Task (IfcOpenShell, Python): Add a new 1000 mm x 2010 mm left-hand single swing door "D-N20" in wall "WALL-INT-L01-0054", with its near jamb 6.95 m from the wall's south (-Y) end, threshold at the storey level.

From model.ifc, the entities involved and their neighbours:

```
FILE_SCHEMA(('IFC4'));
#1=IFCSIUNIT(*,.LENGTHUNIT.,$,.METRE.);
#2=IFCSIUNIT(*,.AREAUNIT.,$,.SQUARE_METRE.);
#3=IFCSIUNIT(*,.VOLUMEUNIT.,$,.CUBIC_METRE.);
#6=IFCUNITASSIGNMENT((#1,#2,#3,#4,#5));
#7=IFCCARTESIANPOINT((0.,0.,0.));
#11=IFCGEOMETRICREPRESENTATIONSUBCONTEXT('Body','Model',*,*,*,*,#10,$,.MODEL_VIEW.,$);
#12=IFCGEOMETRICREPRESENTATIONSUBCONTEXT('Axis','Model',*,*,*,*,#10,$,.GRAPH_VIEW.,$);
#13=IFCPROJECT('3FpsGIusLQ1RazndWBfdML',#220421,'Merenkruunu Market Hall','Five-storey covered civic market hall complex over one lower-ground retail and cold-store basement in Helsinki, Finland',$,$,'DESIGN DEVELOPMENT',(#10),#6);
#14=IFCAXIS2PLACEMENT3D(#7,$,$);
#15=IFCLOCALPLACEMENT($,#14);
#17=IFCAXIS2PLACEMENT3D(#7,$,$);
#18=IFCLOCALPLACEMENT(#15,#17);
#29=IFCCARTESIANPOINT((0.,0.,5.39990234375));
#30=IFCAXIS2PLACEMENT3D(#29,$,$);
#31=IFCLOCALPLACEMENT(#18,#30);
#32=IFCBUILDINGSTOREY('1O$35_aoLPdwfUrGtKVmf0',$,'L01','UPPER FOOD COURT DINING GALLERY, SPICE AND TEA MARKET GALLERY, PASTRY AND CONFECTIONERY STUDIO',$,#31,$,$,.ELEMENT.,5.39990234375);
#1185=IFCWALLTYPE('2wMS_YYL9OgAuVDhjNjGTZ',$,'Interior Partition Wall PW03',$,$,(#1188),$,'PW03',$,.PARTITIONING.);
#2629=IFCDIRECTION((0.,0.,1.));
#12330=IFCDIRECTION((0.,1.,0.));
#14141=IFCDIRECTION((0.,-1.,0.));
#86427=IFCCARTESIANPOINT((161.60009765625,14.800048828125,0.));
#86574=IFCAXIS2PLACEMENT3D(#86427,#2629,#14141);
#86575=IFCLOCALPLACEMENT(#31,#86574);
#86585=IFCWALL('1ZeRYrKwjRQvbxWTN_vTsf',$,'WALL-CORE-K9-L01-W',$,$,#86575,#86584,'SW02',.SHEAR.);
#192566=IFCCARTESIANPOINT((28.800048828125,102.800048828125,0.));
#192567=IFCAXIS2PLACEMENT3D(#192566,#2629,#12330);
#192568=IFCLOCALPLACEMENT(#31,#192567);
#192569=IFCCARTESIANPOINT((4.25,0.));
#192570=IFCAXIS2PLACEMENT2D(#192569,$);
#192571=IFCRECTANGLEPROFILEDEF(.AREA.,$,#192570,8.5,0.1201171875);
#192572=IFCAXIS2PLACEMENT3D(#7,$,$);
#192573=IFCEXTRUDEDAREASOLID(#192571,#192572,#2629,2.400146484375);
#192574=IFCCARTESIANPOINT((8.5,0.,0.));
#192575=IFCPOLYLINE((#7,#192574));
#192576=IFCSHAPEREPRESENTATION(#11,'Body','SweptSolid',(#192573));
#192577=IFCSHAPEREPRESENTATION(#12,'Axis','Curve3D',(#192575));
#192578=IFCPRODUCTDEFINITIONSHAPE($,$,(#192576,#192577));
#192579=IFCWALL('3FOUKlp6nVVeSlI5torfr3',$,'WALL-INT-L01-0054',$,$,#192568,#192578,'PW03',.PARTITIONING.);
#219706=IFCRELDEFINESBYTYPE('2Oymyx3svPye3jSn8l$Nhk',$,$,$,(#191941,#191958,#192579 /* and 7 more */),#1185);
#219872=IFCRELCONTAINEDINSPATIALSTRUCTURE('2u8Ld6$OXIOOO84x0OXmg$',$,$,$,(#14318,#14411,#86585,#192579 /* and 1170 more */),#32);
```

```python
import numpy as np
import ifcopenshell
import ifcopenshell.api.feature
import ifcopenshell.api.geometry
import ifcopenshell.api.root
import ifcopenshell.api.spatial
import ifcopenshell.geom
import ifcopenshell.util.element
import ifcopenshell.util.placement
import ifcopenshell.util.representation
import ifcopenshell.util.shape
import ifcopenshell.util.unit

model = ifcopenshell.open("model.ifc")
unit_scale = ifcopenshell.util.unit.calculate_unit_scale(model)
settings = ifcopenshell.geom.settings()


def volume(element):
    """Net volume in cubic metres, openings subtracted."""
    shape = ifcopenshell.geom.create_shape(settings, element)
    return ifcopenshell.util.shape.get_volume(shape.geometry)


wall = model.by_id(192579)
storey = ifcopenshell.util.element.get_container(wall, ifc_class="IfcBuildingStorey")
context = ifcopenshell.util.representation.get_context(model, "Model", "Body", "MODEL_VIEW")
before = volume(wall)

width, height, from_end, sill = 1, 2.01, 6.95, 0.0  # metres

# The wall runs along its own X axis, and the end named is its -X end.
wall_shape = ifcopenshell.geom.create_shape(settings, wall)
x, y, z = ifcopenshell.util.shape.get_vertices(wall_shape.geometry).T
start = x.min() + from_end
face, thickness = float(y.min()), float(y.max() - y.min())
wall_matrix = ifcopenshell.util.placement.get_local_placement(wall.ObjectPlacement)
level = ifcopenshell.util.placement.get_local_placement(storey.ObjectPlacement)[2, 3]


def in_wall(x, y):
    """Placement at x, y metres in the wall's axes, at sill height."""
    matrix = wall_matrix.copy()
    matrix[:, 3] = wall_matrix @ np.array([x / unit_scale, y / unit_scale, 0.0, 1.0])
    matrix[2, 3] = level + sill / unit_scale
    return matrix


# Opening: a box that overshoots both wall faces by 50 mm.
opening = ifcopenshell.api.root.create_entity(model, ifc_class="IfcOpeningElement", predefined_type="OPENING")
box = ifcopenshell.api.geometry.add_wall_representation(
    model, context=context, length=width, height=height, thickness=thickness + 0.1
)
ifcopenshell.api.geometry.assign_representation(model, product=opening, representation=box)
ifcopenshell.api.geometry.edit_object_placement(model, product=opening, matrix=in_wall(start, face - 0.05), is_si=False)
ifcopenshell.api.feature.add_feature(model, feature=opening, element=wall)

door = ifcopenshell.api.root.create_entity(model, ifc_class="IfcDoor", name="D-N20", predefined_type="DOOR")
door.OverallWidth, door.OverallHeight = width / unit_scale, height / unit_scale
door.OperationType = "SINGLE_SWING_LEFT"
body = ifcopenshell.api.geometry.add_door_representation(
    model,
    context=context,
    overall_width=door.OverallWidth,
    overall_height=door.OverallHeight,
    operation_type="SINGLE_SWING_LEFT",
    lining_properties={"LiningDepth": thickness / unit_scale, "ThresholdDepth": thickness / unit_scale},
)
ifcopenshell.api.geometry.assign_representation(model, product=door, representation=body)
ifcopenshell.api.spatial.assign_container(model, products=[door], relating_structure=storey)
ifcopenshell.api.feature.add_filling(model, opening=opening, element=door)

# The lining spans the wall, so the door starts at the wall face.
ifcopenshell.api.geometry.edit_object_placement(model, product=door, matrix=in_wall(start, face), is_si=False)

after = volume(wall)

print(f"wall volume {before:.3f} -> {after:.3f} m3")

model.write("model_v2.ifc")
```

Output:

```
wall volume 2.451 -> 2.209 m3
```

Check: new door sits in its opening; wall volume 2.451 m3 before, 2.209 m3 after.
